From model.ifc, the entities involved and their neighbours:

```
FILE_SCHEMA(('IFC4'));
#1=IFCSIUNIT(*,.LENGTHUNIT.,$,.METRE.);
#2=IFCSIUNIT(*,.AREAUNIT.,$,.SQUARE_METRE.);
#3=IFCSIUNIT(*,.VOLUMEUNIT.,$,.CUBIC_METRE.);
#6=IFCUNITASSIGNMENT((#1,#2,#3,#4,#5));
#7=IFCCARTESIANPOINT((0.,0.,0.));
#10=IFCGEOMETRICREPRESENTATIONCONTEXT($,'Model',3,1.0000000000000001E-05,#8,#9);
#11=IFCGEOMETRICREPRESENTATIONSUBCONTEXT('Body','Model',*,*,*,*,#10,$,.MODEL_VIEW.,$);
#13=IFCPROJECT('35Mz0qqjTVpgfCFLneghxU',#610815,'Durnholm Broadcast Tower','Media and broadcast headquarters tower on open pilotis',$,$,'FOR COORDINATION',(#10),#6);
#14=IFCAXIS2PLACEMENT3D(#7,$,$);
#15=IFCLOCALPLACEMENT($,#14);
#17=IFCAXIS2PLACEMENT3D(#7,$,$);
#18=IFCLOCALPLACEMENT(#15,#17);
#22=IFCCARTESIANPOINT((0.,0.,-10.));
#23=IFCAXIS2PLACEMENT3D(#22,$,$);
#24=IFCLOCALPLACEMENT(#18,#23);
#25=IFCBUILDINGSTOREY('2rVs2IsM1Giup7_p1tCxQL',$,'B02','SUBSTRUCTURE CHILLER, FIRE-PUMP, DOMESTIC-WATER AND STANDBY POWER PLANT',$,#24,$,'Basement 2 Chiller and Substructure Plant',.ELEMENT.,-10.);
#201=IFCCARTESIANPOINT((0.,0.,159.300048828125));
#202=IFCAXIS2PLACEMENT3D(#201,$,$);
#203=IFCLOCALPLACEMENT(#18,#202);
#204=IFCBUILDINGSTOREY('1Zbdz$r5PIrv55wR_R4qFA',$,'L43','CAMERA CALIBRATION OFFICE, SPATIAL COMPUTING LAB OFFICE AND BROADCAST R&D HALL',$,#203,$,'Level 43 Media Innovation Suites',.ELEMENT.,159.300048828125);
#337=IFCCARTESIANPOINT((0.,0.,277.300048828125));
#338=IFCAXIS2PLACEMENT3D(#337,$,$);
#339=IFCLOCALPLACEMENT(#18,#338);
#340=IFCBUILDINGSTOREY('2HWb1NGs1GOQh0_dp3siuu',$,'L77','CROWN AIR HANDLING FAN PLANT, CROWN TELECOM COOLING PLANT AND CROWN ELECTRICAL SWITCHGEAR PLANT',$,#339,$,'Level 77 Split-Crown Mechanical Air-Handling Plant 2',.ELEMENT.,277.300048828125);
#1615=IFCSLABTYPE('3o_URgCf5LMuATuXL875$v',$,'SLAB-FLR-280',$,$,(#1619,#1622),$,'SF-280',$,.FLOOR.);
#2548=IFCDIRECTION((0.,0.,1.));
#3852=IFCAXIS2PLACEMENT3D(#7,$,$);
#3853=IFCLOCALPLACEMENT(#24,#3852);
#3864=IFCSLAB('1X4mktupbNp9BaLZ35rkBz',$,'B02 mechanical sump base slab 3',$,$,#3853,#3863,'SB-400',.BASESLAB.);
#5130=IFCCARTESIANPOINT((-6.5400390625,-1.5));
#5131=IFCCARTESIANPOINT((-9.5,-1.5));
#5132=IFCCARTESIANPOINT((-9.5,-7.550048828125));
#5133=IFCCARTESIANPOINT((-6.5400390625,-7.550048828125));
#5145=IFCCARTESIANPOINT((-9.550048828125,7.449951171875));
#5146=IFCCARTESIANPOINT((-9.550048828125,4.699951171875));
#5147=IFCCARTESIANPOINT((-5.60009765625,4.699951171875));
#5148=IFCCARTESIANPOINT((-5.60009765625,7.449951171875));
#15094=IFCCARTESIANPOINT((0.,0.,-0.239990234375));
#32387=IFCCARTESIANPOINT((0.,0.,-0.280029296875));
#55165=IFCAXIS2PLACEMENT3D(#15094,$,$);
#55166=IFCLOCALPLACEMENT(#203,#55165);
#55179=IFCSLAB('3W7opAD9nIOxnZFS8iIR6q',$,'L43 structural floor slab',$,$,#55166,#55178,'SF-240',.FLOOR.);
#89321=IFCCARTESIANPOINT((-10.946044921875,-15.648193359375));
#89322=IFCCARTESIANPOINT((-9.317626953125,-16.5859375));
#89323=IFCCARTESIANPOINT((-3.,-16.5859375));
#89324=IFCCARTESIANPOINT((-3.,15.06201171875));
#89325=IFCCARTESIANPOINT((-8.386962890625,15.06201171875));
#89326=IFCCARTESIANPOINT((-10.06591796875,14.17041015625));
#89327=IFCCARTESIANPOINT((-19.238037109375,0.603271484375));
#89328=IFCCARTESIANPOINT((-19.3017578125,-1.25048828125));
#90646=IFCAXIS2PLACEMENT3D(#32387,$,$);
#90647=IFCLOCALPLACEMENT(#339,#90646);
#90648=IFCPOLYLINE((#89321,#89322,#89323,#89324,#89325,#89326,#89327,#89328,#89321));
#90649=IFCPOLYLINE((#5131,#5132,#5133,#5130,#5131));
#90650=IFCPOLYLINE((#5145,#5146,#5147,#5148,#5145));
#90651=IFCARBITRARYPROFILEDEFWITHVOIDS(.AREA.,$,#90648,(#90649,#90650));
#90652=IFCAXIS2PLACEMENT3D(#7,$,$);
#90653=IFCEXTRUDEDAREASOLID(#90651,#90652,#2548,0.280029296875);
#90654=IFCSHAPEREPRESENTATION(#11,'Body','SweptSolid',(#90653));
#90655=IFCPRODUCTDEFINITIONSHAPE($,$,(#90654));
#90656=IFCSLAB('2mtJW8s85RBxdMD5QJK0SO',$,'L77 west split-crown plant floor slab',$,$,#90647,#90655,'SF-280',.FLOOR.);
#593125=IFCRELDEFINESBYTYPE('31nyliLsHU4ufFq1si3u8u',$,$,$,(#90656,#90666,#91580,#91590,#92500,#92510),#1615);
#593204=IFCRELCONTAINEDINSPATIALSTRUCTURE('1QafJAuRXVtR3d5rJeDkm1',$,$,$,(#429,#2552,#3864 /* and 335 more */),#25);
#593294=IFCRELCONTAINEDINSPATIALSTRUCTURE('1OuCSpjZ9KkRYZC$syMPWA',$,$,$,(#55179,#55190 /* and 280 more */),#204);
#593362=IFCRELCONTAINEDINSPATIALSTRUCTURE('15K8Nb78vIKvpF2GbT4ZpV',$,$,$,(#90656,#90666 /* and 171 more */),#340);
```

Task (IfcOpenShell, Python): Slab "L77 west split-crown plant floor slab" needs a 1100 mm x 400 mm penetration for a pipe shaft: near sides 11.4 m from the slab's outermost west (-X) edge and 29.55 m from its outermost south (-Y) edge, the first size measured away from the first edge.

```python
import numpy as np
import ifcopenshell
import ifcopenshell.api.feature
import ifcopenshell.api.geometry
import ifcopenshell.api.root
import ifcopenshell.geom
import ifcopenshell.util.placement
import ifcopenshell.util.representation
import ifcopenshell.util.shape
import ifcopenshell.util.unit

model = ifcopenshell.open("model.ifc")
unit_scale = ifcopenshell.util.unit.calculate_unit_scale(model)
settings = ifcopenshell.geom.settings()


def volume(element):
    """Net volume in cubic metres, openings subtracted."""
    shape = ifcopenshell.geom.create_shape(settings, element)
    return ifcopenshell.util.shape.get_volume(shape.geometry)


slab = model.by_guid("2mtJW8s85RBxdMD5QJK0SO")
before = volume(slab)

# Extent in the slab's own axes, in metres. The edges named are its -X and -Y sides.
slab_shape = ifcopenshell.geom.create_shape(settings, slab)
vertices = ifcopenshell.util.shape.get_vertices(slab_shape.geometry)
x_min, y_min, bottom = vertices.min(axis=0)
top = vertices[:, 2].max()

opening = ifcopenshell.api.root.create_entity(model, ifc_class="IfcOpeningElement", name="Pipe shaft opening", predefined_type="OPENING")
context = ifcopenshell.util.representation.get_context(model, "Model", "Body", "MODEL_VIEW")
width, depth = 1.1, 0.4
outline = [(0.0, 0.0), (width, 0.0), (width, depth), (0.0, depth), (0.0, 0.0)]
# Overshoot both faces by 50 mm so the cut is clean.
shape = ifcopenshell.api.geometry.add_slab_representation(
    model, context=context, depth=top - bottom + 0.1, polyline=outline
)
ifcopenshell.api.geometry.assign_representation(model, product=opening, representation=shape)

matrix = ifcopenshell.util.placement.get_local_placement(slab.ObjectPlacement)
matrix[:, 3] = matrix @ np.append(np.array([x_min + 11.4, y_min + 29.55, bottom - 0.05]) / unit_scale, 1.0)
ifcopenshell.api.geometry.edit_object_placement(model, product=opening, matrix=matrix, is_si=False)
ifcopenshell.api.feature.add_feature(model, feature=opening, element=slab)

after = volume(slab)

print(f"slab volume {before:.3f} -> {after:.3f} m3")

model.write("model_updated.ifc")
```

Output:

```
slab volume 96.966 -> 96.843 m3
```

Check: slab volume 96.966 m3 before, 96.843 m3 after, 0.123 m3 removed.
